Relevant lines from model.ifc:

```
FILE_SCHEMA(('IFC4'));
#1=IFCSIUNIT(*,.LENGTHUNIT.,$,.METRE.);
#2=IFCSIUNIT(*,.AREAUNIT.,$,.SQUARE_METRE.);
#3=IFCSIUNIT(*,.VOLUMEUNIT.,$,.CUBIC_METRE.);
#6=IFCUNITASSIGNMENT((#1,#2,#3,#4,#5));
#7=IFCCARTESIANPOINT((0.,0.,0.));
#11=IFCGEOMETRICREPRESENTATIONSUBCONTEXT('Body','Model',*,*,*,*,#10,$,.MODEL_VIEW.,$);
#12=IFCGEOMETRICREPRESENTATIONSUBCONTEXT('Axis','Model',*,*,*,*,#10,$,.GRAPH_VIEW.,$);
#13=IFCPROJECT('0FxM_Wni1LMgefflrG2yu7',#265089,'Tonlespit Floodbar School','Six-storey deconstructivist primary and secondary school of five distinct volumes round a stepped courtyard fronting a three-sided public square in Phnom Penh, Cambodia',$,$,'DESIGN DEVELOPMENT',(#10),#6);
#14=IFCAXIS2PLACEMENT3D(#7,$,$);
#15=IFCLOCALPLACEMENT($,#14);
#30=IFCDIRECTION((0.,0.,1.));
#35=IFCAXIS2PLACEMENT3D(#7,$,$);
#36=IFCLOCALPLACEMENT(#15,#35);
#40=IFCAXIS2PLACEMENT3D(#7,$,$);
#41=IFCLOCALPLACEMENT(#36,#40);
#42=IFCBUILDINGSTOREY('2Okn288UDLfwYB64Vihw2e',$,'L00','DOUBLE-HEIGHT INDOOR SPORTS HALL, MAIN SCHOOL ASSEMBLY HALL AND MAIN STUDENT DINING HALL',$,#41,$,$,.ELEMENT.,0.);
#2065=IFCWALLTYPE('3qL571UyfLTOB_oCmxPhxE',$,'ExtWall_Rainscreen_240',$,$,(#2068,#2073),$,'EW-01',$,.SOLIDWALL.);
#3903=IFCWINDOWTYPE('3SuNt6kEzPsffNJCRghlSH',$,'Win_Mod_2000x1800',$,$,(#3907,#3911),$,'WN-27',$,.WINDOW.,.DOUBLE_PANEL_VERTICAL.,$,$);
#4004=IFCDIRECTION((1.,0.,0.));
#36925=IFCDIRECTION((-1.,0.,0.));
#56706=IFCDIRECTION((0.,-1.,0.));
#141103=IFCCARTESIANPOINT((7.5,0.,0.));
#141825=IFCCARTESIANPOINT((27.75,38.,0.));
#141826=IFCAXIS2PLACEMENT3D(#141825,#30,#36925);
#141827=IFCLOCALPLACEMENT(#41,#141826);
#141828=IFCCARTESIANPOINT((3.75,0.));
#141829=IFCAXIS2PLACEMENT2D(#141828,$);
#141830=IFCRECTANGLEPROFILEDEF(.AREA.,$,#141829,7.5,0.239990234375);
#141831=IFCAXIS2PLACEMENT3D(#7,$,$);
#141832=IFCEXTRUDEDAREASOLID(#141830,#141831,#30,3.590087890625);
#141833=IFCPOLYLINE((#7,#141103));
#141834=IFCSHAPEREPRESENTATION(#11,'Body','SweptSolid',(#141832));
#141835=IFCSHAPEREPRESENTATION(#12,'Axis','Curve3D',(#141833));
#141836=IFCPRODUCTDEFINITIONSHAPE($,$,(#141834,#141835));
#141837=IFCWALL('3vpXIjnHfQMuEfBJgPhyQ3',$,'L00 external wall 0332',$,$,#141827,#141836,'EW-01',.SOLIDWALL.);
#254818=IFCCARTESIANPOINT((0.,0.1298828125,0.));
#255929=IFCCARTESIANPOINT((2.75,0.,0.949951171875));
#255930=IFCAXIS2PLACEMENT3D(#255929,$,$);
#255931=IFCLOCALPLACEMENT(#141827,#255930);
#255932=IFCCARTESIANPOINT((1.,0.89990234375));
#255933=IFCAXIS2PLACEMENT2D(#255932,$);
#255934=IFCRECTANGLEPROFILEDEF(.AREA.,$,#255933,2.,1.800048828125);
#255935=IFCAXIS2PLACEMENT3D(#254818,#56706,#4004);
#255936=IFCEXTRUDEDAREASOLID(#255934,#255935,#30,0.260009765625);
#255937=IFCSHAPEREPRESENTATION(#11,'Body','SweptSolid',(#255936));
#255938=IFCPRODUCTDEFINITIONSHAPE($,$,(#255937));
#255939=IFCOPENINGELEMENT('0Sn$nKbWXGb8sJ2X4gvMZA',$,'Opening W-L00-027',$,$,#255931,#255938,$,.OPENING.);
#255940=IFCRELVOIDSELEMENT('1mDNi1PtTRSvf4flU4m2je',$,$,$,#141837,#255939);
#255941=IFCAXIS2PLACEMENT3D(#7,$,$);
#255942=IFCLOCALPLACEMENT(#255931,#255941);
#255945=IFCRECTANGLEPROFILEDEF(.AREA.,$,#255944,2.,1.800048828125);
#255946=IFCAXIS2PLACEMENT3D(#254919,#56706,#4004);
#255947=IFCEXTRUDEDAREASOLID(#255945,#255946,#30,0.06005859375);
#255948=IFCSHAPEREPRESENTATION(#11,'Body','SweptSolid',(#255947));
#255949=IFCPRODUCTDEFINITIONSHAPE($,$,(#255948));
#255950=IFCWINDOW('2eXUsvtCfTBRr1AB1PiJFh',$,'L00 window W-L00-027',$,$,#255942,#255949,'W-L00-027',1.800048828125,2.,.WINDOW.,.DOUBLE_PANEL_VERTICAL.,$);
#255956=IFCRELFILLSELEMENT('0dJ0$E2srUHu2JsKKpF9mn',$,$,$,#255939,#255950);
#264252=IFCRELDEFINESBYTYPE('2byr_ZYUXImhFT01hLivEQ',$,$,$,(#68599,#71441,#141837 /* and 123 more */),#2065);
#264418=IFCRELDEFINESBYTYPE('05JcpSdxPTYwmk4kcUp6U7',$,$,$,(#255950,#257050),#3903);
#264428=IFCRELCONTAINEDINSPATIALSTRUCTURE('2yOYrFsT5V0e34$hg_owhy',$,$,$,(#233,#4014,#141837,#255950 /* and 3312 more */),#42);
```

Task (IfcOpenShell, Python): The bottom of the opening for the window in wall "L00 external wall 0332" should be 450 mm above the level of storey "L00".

```python
import numpy as np
import ifcopenshell
import ifcopenshell.api.geometry
import ifcopenshell.geom
import ifcopenshell.util.element
import ifcopenshell.util.placement
import ifcopenshell.util.shape
import ifcopenshell.util.unit

model = ifcopenshell.open("model.ifc")
unit_scale = ifcopenshell.util.unit.calculate_unit_scale(model)

window = model.by_guid("2eXUsvtCfTBRr1AB1PiJFh")
opening = window.FillsVoids[0].RelatingOpeningElement
storey = ifcopenshell.util.element.get_container(window, ifc_class="IfcBuildingStorey")
level = ifcopenshell.util.placement.get_local_placement(storey.ObjectPlacement)[2, 3]

# The opening's origin need not be at the sill, so measure its lowest point.
shape = ifcopenshell.geom.create_shape(ifcopenshell.geom.settings(), opening)
bottom = ifcopenshell.util.shape.get_shape_bottom_elevation(shape, shape.geometry) / unit_scale
dz = level + 0.45 - bottom

shift = np.array([0.0, 0.0, dz])
# The window is placed relative to its opening, so it follows when the opening moves.
matrix = ifcopenshell.util.placement.get_local_placement(opening.ObjectPlacement)
matrix[:3, 3] += shift
ifcopenshell.api.geometry.edit_object_placement(
    model, product=opening, matrix=matrix, is_si=False, should_transform_children=True
)

print(f"moved by {dz * unit_scale:+.3f} m")

model.write("model-out.ifc")
```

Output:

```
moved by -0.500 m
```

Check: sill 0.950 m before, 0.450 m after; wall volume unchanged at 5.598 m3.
